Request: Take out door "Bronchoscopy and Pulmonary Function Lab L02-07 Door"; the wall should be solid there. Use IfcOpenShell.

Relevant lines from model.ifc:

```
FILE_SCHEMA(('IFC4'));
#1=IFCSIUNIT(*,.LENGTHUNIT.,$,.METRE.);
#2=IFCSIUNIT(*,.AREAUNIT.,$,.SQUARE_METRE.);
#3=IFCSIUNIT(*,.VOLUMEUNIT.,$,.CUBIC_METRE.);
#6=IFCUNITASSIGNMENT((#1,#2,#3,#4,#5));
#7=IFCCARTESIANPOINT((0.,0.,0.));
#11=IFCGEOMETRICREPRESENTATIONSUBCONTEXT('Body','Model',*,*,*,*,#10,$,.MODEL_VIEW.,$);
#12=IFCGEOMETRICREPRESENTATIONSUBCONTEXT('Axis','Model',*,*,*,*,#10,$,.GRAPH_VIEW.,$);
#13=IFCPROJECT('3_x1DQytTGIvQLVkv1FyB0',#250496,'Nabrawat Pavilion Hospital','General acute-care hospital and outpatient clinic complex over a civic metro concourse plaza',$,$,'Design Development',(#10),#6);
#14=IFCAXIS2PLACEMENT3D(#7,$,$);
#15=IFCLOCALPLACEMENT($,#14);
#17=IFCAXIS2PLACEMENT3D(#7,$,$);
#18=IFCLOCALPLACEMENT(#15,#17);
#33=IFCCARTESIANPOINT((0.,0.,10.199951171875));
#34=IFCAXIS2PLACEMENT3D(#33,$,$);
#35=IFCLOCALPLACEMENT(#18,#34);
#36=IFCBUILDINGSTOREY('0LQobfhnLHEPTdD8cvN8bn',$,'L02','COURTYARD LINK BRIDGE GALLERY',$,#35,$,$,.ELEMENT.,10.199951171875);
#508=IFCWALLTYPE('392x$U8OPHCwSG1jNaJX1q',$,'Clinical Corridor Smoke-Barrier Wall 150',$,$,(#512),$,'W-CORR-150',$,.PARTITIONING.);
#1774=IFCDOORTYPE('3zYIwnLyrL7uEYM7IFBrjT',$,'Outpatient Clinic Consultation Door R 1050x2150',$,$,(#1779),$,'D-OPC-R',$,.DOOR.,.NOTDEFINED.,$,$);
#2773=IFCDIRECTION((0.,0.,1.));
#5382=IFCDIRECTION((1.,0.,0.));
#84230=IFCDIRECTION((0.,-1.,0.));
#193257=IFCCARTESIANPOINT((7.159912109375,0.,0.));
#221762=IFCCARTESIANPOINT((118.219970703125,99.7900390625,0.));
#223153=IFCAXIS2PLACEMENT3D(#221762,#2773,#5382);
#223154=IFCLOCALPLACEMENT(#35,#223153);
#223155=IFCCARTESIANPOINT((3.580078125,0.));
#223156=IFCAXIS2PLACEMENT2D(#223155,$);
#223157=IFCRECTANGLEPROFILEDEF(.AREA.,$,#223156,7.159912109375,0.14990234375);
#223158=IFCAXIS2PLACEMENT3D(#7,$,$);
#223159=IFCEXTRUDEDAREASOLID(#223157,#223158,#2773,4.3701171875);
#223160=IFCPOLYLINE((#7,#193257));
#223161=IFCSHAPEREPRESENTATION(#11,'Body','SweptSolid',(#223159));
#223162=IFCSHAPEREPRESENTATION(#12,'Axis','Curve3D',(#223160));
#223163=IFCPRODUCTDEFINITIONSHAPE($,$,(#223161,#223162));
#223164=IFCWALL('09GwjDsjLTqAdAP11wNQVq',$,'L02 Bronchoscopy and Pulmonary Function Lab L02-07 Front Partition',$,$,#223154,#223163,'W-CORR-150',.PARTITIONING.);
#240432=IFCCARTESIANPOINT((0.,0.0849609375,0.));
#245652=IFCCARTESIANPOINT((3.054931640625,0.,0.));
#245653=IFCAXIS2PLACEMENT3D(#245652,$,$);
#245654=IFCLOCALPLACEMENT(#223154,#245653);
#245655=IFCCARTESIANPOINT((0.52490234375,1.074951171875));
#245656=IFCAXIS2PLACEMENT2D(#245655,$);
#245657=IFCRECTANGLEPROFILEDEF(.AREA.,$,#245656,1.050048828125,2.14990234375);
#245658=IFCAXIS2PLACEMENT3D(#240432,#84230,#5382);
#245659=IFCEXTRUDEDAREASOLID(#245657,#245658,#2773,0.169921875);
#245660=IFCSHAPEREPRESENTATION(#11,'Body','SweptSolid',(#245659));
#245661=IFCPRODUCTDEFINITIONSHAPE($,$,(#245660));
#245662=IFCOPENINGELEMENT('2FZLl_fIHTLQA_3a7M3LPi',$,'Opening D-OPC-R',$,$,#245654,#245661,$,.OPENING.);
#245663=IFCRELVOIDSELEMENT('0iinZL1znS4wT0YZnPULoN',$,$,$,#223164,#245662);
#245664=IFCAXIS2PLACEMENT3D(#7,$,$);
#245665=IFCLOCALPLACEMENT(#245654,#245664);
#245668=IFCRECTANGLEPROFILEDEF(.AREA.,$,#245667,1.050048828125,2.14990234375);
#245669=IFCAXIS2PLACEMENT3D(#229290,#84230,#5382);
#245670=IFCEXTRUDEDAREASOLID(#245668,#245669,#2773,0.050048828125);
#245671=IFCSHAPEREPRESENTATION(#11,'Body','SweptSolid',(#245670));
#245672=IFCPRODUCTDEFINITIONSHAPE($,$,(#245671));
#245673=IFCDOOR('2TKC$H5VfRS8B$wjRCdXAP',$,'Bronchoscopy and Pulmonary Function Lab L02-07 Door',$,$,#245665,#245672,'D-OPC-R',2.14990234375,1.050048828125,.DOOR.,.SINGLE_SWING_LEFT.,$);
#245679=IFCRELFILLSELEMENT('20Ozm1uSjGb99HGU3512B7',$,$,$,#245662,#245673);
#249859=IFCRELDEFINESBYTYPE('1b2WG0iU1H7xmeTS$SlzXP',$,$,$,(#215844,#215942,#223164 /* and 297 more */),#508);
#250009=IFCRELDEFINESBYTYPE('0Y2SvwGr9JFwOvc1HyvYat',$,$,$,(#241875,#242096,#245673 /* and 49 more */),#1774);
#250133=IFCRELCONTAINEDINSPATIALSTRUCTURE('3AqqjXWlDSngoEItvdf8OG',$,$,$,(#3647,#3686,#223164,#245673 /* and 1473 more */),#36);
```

```python
import ifcopenshell
import ifcopenshell.api.feature
import ifcopenshell.api.root
import ifcopenshell.geom
import ifcopenshell.util.shape

model = ifcopenshell.open("model.ifc")
settings = ifcopenshell.geom.settings()


def volume(element):
    """Net volume in cubic metres, openings subtracted."""
    shape = ifcopenshell.geom.create_shape(settings, element)
    return ifcopenshell.util.shape.get_volume(shape.geometry)


door = model.by_guid("2TKC$H5VfRS8B$wjRCdXAP")
opening = door.FillsVoids[0].RelatingOpeningElement
wall = opening.VoidsElements[0].RelatingBuildingElement
before = volume(wall)

ifcopenshell.api.root.remove_product(model, product=door)
ifcopenshell.api.feature.remove_feature(model, feature=opening)

after = volume(wall)

print(f"wall volume {before:.3f} -> {after:.3f} m3")

model.write("model_updated.ifc")
```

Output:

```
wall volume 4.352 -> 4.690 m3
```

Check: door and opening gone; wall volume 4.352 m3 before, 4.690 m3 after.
